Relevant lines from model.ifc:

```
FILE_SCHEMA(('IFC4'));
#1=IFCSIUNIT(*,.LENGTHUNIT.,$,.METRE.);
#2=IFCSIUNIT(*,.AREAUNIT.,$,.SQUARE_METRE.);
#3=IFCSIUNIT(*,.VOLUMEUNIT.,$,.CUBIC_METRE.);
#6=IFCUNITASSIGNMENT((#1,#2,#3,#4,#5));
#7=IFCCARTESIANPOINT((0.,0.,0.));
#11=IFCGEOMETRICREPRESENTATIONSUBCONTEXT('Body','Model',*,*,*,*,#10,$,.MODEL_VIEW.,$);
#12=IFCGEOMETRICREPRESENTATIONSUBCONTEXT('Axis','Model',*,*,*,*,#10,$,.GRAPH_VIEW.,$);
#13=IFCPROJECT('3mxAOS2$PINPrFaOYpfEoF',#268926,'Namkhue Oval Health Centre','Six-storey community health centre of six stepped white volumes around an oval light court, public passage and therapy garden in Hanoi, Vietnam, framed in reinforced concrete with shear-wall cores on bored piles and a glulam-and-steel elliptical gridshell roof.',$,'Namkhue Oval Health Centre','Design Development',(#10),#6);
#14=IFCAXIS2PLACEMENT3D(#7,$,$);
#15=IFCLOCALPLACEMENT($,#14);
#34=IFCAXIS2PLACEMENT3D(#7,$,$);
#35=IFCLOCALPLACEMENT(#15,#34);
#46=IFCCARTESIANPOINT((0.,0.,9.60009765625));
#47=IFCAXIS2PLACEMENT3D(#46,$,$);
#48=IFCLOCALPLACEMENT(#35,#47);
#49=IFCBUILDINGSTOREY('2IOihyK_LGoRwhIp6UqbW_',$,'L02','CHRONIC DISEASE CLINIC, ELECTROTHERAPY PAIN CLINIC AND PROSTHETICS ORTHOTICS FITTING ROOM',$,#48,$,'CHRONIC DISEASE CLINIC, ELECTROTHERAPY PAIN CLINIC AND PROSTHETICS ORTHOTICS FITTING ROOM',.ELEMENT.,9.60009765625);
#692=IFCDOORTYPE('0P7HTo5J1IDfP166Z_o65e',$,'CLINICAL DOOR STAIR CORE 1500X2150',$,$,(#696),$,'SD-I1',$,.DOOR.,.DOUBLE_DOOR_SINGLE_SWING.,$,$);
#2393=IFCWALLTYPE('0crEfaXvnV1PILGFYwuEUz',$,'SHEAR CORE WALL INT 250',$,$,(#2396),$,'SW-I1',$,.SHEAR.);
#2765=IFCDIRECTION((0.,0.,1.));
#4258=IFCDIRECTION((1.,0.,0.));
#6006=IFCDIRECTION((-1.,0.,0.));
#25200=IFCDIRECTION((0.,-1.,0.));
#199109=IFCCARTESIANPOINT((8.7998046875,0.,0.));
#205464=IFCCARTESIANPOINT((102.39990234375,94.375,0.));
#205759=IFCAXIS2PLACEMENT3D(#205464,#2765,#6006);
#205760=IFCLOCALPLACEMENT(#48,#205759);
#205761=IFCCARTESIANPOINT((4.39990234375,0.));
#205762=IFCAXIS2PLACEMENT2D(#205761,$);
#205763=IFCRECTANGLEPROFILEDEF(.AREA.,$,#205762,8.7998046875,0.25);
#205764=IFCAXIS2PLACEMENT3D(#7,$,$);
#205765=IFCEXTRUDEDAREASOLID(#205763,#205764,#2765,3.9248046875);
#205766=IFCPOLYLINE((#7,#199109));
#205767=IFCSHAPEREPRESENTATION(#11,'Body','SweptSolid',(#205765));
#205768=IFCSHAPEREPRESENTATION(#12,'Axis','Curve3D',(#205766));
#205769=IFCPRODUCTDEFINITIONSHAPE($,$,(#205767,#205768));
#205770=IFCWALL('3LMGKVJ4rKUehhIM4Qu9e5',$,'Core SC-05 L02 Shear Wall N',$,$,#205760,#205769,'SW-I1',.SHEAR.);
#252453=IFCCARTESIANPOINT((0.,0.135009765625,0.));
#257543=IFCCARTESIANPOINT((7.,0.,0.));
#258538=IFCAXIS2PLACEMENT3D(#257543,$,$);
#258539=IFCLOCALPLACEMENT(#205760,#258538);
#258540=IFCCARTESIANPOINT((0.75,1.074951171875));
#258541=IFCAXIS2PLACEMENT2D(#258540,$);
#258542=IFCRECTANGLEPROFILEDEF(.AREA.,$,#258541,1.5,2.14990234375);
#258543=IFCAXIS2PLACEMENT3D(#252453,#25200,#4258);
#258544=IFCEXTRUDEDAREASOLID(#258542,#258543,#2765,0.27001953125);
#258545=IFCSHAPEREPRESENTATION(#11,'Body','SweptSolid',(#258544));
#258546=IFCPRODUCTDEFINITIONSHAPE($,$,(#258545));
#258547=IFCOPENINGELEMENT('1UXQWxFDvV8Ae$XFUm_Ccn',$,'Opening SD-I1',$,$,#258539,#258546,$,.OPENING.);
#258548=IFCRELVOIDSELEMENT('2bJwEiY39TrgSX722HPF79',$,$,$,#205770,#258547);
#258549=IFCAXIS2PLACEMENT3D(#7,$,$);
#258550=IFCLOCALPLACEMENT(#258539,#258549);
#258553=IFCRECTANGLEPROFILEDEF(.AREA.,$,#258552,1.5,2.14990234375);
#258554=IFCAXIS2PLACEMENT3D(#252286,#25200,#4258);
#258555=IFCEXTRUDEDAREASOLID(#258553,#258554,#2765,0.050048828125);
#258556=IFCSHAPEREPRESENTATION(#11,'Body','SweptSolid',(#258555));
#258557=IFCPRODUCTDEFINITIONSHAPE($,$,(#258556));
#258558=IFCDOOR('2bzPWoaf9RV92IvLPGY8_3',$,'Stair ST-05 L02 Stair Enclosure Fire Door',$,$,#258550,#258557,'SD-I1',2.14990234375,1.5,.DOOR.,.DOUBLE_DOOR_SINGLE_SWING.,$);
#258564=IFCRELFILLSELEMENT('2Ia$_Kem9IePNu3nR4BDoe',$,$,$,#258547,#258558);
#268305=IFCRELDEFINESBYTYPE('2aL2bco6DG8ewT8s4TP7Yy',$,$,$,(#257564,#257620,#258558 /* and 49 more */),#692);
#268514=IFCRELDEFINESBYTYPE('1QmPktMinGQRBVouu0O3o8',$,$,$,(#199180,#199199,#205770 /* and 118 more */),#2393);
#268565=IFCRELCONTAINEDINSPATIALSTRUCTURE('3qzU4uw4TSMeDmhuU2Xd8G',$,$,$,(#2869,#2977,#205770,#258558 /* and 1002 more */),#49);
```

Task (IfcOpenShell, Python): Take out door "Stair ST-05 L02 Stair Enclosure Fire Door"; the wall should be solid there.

```python
import ifcopenshell
import ifcopenshell.api.feature
import ifcopenshell.api.root
import ifcopenshell.geom
import ifcopenshell.util.shape

model = ifcopenshell.open("model.ifc")
settings = ifcopenshell.geom.settings()


def volume(element):
    """Net volume in cubic metres, openings subtracted."""
    shape = ifcopenshell.geom.create_shape(settings, element)
    return ifcopenshell.util.shape.get_volume(shape.geometry)


door = model.by_guid("2bzPWoaf9RV92IvLPGY8_3")
opening = door.FillsVoids[0].RelatingOpeningElement
wall = opening.VoidsElements[0].RelatingBuildingElement
before = volume(wall)

ifcopenshell.api.root.remove_product(model, product=door)
ifcopenshell.api.feature.remove_feature(model, feature=opening)

after = volume(wall)

print(f"wall volume {before:.3f} -> {after:.3f} m3")

model.write("model_edited.ifc")
```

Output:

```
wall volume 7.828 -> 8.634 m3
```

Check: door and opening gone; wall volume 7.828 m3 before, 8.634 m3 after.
